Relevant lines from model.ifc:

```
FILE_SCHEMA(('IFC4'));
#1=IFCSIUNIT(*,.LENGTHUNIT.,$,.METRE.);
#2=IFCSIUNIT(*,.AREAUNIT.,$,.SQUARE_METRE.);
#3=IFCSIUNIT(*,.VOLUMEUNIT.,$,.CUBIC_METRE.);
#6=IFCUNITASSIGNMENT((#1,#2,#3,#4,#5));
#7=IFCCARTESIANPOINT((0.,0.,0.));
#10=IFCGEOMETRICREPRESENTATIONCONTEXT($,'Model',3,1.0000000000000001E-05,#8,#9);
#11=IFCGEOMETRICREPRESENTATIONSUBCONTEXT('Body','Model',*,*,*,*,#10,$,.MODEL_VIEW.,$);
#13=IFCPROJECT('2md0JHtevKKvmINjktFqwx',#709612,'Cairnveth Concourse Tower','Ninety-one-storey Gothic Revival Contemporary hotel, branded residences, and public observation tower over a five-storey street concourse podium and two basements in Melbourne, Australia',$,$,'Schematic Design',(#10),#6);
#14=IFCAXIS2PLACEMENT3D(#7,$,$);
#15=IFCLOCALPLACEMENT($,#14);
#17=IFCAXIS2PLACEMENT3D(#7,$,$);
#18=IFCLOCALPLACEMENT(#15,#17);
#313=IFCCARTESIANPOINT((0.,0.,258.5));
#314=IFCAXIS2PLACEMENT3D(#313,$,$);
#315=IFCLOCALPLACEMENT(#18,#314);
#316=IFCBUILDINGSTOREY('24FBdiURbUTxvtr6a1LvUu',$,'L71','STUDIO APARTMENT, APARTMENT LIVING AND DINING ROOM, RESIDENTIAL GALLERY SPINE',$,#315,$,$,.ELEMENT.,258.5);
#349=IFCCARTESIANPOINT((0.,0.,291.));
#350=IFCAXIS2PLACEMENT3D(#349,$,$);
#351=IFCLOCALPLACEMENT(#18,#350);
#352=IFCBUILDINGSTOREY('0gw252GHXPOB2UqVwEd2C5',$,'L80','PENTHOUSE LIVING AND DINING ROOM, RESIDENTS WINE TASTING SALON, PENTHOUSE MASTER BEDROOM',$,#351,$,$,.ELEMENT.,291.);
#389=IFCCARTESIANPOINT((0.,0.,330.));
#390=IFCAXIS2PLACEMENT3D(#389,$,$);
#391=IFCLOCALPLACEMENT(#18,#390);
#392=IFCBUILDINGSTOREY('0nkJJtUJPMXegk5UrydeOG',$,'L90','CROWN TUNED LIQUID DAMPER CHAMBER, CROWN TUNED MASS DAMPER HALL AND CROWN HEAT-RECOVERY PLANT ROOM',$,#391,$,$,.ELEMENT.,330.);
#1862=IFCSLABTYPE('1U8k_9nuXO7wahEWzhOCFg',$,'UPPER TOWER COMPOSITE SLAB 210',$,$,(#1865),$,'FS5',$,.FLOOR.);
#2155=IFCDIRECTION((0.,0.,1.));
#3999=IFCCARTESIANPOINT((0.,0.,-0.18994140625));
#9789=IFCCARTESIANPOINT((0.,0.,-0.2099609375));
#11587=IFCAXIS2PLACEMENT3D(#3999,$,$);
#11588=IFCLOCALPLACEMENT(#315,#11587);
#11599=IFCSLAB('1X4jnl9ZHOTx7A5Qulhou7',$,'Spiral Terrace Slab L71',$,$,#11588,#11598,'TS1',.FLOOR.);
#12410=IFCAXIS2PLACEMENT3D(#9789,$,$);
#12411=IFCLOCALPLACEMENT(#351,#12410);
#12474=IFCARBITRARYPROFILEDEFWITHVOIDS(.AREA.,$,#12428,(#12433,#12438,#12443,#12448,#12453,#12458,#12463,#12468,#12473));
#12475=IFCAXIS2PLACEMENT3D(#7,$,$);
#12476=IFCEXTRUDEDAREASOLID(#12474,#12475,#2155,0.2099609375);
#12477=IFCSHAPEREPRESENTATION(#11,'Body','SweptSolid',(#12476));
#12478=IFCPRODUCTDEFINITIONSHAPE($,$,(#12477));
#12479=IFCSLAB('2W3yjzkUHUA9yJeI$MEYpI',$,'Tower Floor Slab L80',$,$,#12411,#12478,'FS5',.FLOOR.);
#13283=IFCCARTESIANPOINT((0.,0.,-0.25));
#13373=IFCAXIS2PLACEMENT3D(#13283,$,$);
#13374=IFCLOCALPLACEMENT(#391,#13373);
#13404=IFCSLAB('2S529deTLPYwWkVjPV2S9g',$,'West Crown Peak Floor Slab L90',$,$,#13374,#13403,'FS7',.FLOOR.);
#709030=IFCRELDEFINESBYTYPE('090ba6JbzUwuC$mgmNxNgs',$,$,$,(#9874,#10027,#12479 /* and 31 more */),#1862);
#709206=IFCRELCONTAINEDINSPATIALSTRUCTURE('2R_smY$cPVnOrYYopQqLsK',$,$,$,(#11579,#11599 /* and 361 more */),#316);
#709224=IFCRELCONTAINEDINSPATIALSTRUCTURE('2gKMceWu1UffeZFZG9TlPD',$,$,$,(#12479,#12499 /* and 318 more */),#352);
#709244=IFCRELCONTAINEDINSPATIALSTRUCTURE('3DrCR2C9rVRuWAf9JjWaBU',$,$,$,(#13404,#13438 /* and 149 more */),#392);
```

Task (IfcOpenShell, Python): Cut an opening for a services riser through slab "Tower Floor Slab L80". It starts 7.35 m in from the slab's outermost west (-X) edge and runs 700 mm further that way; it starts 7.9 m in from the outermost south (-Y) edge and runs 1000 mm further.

```python
import numpy as np
import ifcopenshell
import ifcopenshell.api.feature
import ifcopenshell.api.geometry
import ifcopenshell.api.root
import ifcopenshell.geom
import ifcopenshell.util.placement
import ifcopenshell.util.representation
import ifcopenshell.util.shape
import ifcopenshell.util.unit

model = ifcopenshell.open("model.ifc")
unit_scale = ifcopenshell.util.unit.calculate_unit_scale(model)
settings = ifcopenshell.geom.settings()


def volume(element):
    """Net volume in cubic metres, openings subtracted."""
    shape = ifcopenshell.geom.create_shape(settings, element)
    return ifcopenshell.util.shape.get_volume(shape.geometry)


slab = model.by_id(12479)
before = volume(slab)

# Extent in the slab's own axes, in metres. The edges named are its -X and -Y sides.
slab_shape = ifcopenshell.geom.create_shape(settings, slab)
vertices = ifcopenshell.util.shape.get_vertices(slab_shape.geometry)
x_min, y_min, bottom = vertices.min(axis=0)
top = vertices[:, 2].max()

opening = ifcopenshell.api.root.create_entity(model, ifc_class="IfcOpeningElement", name="Services riser opening", predefined_type="OPENING")
context = ifcopenshell.util.representation.get_context(model, "Model", "Body", "MODEL_VIEW")
width, depth = 0.7, 1
outline = [(0.0, 0.0), (width, 0.0), (width, depth), (0.0, depth), (0.0, 0.0)]
# Overshoot both faces by 50 mm so the cut is clean.
shape = ifcopenshell.api.geometry.add_slab_representation(
    model, context=context, depth=top - bottom + 0.1, polyline=outline
)
ifcopenshell.api.geometry.assign_representation(model, product=opening, representation=shape)

matrix = ifcopenshell.util.placement.get_local_placement(slab.ObjectPlacement)
matrix[:, 3] = matrix @ np.append(np.array([x_min + 7.35, y_min + 7.9, bottom - 0.05]) / unit_scale, 1.0)
ifcopenshell.api.geometry.edit_object_placement(model, product=opening, matrix=matrix, is_si=False)
ifcopenshell.api.feature.add_feature(model, feature=opening, element=slab)

after = volume(slab)

print(f"slab volume {before:.3f} -> {after:.3f} m3")

model.write("model_updated.ifc")
```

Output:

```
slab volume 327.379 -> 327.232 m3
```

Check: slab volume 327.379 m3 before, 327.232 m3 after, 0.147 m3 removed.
